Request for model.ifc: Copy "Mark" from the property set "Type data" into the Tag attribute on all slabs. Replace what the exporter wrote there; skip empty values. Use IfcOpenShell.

First a look at what the model holds.

```python
import ifcopenshell
import ifcopenshell.util.element

model = ifcopenshell.open("model.ifc")
print(model.schema)
slabs = model.by_type("IfcSlab")
print(len(slabs), "slabs")
for e in slabs[:8]:
    source = ifcopenshell.util.element.get_pset(e, "Type data", "Mark")
    target = e.Tag
    print(e.id(), repr(source), repr(target), sep=" | ")
```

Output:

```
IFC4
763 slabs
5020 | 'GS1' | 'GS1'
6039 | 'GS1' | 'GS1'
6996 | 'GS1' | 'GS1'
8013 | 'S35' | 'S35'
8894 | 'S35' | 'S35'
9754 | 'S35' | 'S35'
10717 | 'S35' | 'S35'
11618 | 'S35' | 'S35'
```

```python
import ifcopenshell
import ifcopenshell.util.element

model = ifcopenshell.open("model.ifc")

count = 0
for e in model.by_type("IfcSlab"):
    value = ifcopenshell.util.element.get_pset(e, "Type data", "Mark")
    current = e.Tag
    if not value or not value.strip() or current == value:
        continue
    e.Tag = value
    count += 1

print(count, "slabs updated")

model.write("model_edited.ifc")
```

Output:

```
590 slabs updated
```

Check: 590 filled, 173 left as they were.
